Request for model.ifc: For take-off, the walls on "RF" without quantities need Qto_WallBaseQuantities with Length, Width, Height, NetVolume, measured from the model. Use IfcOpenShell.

First a look at what the model holds.

```python
import ifcopenshell
import ifcopenshell.util.element
import ifcopenshell.util.unit

model = ifcopenshell.open("model.ifc")
print(model.schema)
for unit_type in ("LENGTHUNIT", "AREAUNIT", "VOLUMEUNIT"):
    print(unit_type, ifcopenshell.util.unit.calculate_unit_scale(model, unit_type))
storey = next(s for s in model.by_type("IfcBuildingStorey") if s.Name == "RF")
walls = [e for e in ifcopenshell.util.element.get_decomposition(storey) if e.is_a("IfcWall")]
for e in sorted(walls, key=lambda e: e.id()):
    print(e.id(), e.is_a(), e.Name, list(ifcopenshell.util.element.get_psets(e, qtos_only=True)), sep=" | ")
```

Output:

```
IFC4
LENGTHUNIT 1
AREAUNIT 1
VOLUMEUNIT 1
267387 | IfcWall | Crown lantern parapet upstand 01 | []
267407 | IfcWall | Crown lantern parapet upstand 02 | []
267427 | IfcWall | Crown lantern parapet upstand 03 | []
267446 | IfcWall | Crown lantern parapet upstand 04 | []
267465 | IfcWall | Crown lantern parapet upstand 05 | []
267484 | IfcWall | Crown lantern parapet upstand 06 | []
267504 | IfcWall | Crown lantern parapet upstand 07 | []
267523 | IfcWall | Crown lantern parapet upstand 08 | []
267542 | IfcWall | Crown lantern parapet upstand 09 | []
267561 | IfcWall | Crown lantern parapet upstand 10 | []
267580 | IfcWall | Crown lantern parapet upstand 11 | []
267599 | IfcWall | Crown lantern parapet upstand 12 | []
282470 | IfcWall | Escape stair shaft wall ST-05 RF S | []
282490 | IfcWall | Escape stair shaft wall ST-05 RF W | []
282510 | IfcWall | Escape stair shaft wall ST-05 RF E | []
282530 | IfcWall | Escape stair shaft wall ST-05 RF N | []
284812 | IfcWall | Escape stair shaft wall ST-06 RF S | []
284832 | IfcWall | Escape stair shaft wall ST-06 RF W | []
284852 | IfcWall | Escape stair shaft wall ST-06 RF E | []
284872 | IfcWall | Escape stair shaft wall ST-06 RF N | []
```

```python
import ifcopenshell
import ifcopenshell.api.pset
import ifcopenshell.geom
import ifcopenshell.util.element
import ifcopenshell.util.shape
import ifcopenshell.util.unit

model = ifcopenshell.open("model.ifc")
unit_scale = ifcopenshell.util.unit.calculate_unit_scale(model)
volume_scale = ifcopenshell.util.unit.calculate_unit_scale(model, "VOLUMEUNIT")
settings = ifcopenshell.geom.settings()

storey = next(s for s in model.by_type("IfcBuildingStorey") if s.Name == "RF")
walls = [e for e in ifcopenshell.util.element.get_decomposition(storey) if e.is_a("IfcWall")]

for e in sorted(walls, key=lambda e: e.id()):
    if ifcopenshell.util.element.get_psets(e, qtos_only=True, should_inherit=False):
        continue
    # Geometry comes back in metres, in the element's own axes.
    shape = ifcopenshell.geom.create_shape(settings, e)
    values = {
        "Length": ifcopenshell.util.shape.get_x(shape.geometry) / unit_scale,
        "Width": ifcopenshell.util.shape.get_y(shape.geometry) / unit_scale,
        "Height": ifcopenshell.util.shape.get_z(shape.geometry) / unit_scale,
        "NetVolume": ifcopenshell.util.shape.get_volume(shape.geometry) / volume_scale,
    }
    qto = ifcopenshell.api.pset.add_qto(model, product=e, name="Qto_WallBaseQuantities")
    ifcopenshell.api.pset.edit_qto(model, qto=qto, properties=values)
    print(e.id(), {k: round(v, 3) for k, v in values.items()})

model.write("model_updated.ifc")
```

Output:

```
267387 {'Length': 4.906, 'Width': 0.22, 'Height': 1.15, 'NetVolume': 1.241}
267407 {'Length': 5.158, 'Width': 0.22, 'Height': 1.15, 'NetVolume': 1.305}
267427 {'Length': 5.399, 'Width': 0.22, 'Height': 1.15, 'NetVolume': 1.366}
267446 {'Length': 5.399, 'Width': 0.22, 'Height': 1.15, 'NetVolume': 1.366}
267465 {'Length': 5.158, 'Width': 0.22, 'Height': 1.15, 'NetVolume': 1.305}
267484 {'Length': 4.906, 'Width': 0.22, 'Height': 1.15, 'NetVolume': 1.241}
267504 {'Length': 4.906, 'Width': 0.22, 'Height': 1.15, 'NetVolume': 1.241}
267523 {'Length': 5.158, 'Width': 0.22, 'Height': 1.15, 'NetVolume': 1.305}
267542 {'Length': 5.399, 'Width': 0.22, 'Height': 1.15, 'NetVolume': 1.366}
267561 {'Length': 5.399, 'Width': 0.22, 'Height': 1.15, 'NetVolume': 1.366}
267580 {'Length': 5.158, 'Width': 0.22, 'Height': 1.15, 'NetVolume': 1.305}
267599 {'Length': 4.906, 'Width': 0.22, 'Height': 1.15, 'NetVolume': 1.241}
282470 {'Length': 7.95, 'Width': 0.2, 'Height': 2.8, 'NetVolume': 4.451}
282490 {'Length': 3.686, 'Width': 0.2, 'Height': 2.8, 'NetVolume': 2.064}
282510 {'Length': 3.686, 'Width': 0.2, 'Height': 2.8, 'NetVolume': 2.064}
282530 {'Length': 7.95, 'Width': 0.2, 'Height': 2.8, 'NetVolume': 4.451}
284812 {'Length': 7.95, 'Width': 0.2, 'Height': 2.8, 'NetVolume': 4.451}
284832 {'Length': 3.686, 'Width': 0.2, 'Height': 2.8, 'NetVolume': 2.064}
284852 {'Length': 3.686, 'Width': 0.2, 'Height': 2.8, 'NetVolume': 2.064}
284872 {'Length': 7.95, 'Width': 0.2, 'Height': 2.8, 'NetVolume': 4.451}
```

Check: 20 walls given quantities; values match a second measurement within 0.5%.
